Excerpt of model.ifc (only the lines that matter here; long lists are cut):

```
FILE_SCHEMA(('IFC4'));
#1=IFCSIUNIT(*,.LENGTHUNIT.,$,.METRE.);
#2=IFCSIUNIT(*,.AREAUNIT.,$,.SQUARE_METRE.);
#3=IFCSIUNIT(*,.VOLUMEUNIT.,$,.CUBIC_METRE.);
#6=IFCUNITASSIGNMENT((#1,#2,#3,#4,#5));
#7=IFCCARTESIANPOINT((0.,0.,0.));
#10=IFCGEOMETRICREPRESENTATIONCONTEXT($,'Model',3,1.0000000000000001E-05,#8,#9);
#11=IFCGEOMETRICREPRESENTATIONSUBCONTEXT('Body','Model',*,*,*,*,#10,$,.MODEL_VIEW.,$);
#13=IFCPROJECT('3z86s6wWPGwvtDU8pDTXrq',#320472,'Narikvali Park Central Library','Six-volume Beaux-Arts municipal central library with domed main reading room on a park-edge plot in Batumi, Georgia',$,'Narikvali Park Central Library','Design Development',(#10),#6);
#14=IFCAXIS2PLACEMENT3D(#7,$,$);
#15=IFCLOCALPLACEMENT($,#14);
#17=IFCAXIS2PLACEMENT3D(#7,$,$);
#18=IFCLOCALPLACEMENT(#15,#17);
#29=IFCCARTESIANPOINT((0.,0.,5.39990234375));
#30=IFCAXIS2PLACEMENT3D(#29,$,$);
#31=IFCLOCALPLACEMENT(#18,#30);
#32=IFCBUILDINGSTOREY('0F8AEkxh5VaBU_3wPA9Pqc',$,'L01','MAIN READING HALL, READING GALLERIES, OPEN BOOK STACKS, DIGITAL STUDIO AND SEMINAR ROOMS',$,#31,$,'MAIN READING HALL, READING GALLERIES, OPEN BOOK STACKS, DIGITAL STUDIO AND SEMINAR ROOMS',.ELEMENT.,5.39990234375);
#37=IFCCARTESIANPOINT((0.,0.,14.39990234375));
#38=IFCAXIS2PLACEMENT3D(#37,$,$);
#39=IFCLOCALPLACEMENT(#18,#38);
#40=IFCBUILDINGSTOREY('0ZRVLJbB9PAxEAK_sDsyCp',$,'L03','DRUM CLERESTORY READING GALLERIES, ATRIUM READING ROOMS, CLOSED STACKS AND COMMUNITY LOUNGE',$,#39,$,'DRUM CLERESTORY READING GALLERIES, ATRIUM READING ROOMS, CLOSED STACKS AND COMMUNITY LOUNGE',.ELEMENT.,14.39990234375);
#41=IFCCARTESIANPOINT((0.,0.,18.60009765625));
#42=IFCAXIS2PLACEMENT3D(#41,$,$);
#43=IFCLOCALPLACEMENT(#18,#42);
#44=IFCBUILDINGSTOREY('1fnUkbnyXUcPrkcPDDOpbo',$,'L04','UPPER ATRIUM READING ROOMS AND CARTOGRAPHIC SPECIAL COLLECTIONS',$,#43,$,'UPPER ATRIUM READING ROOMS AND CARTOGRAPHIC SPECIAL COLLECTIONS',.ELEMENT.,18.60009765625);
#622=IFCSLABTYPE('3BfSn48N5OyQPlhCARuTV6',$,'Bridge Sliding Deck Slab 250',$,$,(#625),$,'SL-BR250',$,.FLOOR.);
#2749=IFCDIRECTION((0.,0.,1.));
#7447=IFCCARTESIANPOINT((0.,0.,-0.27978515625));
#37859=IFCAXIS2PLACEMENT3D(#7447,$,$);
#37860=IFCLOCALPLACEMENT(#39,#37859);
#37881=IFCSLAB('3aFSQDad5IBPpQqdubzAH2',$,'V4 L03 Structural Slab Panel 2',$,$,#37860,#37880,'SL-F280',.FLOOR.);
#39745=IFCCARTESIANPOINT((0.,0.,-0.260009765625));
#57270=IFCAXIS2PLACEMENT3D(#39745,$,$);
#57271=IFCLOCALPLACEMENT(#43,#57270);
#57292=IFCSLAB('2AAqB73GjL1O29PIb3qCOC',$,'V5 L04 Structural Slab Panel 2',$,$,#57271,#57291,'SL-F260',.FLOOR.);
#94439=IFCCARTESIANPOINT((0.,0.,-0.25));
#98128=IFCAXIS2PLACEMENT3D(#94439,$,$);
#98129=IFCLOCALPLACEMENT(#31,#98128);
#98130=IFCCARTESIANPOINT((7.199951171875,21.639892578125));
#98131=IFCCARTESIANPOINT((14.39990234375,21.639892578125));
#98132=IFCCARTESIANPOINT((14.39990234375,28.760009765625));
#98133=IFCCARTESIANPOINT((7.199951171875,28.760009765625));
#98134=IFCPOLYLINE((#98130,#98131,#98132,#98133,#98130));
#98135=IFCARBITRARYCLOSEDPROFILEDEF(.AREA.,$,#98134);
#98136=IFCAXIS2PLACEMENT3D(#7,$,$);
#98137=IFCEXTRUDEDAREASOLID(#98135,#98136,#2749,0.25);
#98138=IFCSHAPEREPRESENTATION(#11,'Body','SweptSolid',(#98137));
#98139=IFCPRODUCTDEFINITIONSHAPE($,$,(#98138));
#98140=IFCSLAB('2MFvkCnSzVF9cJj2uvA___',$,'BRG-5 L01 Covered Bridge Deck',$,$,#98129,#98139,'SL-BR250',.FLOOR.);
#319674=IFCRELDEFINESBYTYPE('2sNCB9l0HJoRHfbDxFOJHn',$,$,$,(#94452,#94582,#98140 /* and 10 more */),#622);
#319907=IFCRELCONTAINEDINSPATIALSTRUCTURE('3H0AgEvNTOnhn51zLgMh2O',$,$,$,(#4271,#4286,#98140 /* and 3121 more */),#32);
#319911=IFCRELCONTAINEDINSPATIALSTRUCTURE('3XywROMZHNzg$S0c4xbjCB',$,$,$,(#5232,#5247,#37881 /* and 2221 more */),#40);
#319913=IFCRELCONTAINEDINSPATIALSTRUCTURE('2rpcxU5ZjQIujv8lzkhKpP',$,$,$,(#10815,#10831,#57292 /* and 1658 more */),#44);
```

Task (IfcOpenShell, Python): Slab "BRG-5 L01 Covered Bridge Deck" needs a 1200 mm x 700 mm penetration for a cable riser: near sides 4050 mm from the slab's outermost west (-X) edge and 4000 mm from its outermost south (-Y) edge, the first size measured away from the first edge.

```python
import numpy as np
import ifcopenshell
import ifcopenshell.api.feature
import ifcopenshell.api.geometry
import ifcopenshell.api.root
import ifcopenshell.geom
import ifcopenshell.util.placement
import ifcopenshell.util.representation
import ifcopenshell.util.shape
import ifcopenshell.util.unit

model = ifcopenshell.open("model.ifc")
unit_scale = ifcopenshell.util.unit.calculate_unit_scale(model)
settings = ifcopenshell.geom.settings()


def volume(element):
    """Net volume in cubic metres, openings subtracted."""
    shape = ifcopenshell.geom.create_shape(settings, element)
    return ifcopenshell.util.shape.get_volume(shape.geometry)


slab = model.by_guid("2MFvkCnSzVF9cJj2uvA___")
before = volume(slab)

# Extent in the slab's own axes, in metres. The edges named are its -X and -Y sides.
slab_shape = ifcopenshell.geom.create_shape(settings, slab)
vertices = ifcopenshell.util.shape.get_vertices(slab_shape.geometry)
x_min, y_min, bottom = vertices.min(axis=0)
top = vertices[:, 2].max()

opening = ifcopenshell.api.root.create_entity(model, ifc_class="IfcOpeningElement", name="Cable riser opening", predefined_type="OPENING")
context = ifcopenshell.util.representation.get_context(model, "Model", "Body", "MODEL_VIEW")
width, depth = 1.2, 0.7
outline = [(0.0, 0.0), (width, 0.0), (width, depth), (0.0, depth), (0.0, 0.0)]
# Overshoot both faces by 50 mm so the cut is clean.
shape = ifcopenshell.api.geometry.add_slab_representation(
    model, context=context, depth=top - bottom + 0.1, polyline=outline
)
ifcopenshell.api.geometry.assign_representation(model, product=opening, representation=shape)

matrix = ifcopenshell.util.placement.get_local_placement(slab.ObjectPlacement)
matrix[:, 3] = matrix @ np.append(np.array([x_min + 4.05, y_min + 4, bottom - 0.05]) / unit_scale, 1.0)
ifcopenshell.api.geometry.edit_object_placement(model, product=opening, matrix=matrix, is_si=False)
ifcopenshell.api.feature.add_feature(model, feature=opening, element=slab)

after = volume(slab)

print(f"slab volume {before:.3f} -> {after:.3f} m3")

model.write("model-out.ifc")
```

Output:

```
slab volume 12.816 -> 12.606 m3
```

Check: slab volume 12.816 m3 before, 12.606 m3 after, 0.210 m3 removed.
